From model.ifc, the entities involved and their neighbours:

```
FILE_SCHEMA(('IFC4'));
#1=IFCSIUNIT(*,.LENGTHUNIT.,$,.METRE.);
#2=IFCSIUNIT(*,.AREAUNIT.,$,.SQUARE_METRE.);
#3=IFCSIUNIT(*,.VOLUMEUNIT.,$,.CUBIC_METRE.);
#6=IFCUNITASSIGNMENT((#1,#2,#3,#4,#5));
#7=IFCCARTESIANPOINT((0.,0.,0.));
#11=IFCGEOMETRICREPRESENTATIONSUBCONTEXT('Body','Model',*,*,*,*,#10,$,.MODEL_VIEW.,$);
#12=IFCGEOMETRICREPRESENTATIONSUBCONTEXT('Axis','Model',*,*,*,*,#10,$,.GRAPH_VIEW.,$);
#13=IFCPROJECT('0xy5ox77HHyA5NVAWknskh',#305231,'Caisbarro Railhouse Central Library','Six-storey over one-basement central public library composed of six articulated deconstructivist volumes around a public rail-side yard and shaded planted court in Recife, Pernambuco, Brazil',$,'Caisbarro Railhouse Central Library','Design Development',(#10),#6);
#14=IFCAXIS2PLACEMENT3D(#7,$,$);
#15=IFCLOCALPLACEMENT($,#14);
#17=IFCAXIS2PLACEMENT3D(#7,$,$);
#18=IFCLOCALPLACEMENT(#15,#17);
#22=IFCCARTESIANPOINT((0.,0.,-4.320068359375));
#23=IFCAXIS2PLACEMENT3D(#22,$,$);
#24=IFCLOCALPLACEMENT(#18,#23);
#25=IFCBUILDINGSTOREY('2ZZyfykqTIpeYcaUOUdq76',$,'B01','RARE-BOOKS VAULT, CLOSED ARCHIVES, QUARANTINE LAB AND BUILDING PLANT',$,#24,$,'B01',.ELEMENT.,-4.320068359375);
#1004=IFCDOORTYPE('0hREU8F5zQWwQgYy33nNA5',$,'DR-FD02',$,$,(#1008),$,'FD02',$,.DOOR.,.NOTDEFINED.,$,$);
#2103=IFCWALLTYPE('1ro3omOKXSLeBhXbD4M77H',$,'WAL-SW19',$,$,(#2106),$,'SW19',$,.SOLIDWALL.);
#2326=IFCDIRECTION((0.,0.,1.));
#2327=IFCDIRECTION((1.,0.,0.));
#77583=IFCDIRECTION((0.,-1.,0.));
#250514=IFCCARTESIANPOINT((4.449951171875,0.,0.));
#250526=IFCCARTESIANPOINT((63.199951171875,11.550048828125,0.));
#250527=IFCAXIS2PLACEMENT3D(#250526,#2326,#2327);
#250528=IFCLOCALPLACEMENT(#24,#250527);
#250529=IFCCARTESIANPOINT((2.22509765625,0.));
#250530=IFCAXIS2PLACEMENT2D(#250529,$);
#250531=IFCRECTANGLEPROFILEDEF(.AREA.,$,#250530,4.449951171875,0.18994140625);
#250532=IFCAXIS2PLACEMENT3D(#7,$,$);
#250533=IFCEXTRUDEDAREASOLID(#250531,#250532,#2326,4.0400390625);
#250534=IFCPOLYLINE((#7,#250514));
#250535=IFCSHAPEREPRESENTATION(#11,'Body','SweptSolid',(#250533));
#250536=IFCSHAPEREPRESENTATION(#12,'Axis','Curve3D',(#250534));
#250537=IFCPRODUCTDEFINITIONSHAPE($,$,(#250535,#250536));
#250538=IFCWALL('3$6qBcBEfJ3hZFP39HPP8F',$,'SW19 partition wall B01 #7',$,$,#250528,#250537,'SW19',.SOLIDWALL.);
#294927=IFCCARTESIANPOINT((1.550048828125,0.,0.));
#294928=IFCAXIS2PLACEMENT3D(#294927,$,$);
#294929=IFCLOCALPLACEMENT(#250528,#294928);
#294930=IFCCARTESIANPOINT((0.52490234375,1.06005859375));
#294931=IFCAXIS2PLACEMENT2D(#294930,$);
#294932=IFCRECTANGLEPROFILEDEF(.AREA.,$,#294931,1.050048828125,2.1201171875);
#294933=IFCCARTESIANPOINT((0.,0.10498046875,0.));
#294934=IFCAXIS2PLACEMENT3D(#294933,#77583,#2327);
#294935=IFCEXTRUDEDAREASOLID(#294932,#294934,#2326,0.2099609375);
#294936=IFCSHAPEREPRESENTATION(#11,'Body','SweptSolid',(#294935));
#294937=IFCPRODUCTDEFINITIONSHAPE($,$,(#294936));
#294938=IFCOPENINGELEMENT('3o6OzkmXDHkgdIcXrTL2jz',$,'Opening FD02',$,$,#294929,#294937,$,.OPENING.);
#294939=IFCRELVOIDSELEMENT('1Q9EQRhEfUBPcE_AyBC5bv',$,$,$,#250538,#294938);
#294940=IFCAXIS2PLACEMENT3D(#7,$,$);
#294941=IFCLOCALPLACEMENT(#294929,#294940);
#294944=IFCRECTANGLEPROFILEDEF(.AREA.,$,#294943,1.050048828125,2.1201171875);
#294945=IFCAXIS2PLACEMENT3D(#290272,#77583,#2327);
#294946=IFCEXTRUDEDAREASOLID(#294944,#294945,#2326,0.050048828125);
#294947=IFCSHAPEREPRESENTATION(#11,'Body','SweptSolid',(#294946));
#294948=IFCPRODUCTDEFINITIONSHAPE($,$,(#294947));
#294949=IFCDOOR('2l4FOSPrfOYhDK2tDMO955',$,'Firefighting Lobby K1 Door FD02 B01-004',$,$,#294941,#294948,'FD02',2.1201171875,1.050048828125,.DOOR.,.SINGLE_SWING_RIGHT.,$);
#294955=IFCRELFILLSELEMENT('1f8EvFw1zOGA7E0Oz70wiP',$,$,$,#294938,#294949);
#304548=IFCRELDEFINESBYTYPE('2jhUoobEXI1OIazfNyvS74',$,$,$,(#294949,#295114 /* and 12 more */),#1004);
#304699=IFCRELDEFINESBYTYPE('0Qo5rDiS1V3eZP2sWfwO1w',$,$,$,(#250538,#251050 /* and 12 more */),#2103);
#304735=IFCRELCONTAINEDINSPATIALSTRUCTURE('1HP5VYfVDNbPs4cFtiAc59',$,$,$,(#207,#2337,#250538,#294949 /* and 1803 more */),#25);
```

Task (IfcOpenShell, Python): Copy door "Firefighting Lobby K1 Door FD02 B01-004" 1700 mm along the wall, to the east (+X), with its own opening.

```python
import ifcopenshell
import ifcopenshell.api.feature
import ifcopenshell.api.geometry
import ifcopenshell.api.root
import ifcopenshell.geom
import ifcopenshell.util.element
import ifcopenshell.util.placement
import ifcopenshell.util.shape
import ifcopenshell.util.unit

model = ifcopenshell.open("model.ifc")
unit_scale = ifcopenshell.util.unit.calculate_unit_scale(model)
settings = ifcopenshell.geom.settings()


def volume(element):
    """Net volume in cubic metres, openings subtracted."""
    shape = ifcopenshell.geom.create_shape(settings, element)
    return ifcopenshell.util.shape.get_volume(shape.geometry)


door = model.by_guid("2l4FOSPrfOYhDK2tDMO955")
opening = door.FillsVoids[0].RelatingOpeningElement
wall = opening.VoidsElements[0].RelatingBuildingElement
before = volume(wall)
shift = ifcopenshell.util.placement.get_local_placement(wall.ObjectPlacement)[:3, 0] * 1.7 / unit_scale

# copy_class copies the void relationship, type, container and properties, but no geometry.
new_opening = ifcopenshell.api.root.copy_class(model, product=opening)
new_opening.Representation = ifcopenshell.util.element.copy_deep(
    model, opening.Representation, exclude=["IfcGeometricRepresentationContext", "IfcRepresentationMap"]
)
new_door = ifcopenshell.api.root.copy_class(model, product=door)
new_door.Representation = ifcopenshell.util.element.copy_deep(
    model, door.Representation, exclude=["IfcGeometricRepresentationContext", "IfcRepresentationMap"]
)
new_door.Tag = None
ifcopenshell.api.feature.add_filling(model, opening=new_opening, element=new_door)

for old, new in ((opening, new_opening), (door, new_door)):
    matrix = ifcopenshell.util.placement.get_local_placement(old.ObjectPlacement)
    matrix[:3, 3] += shift
    ifcopenshell.api.geometry.edit_object_placement(model, product=new, matrix=matrix, is_si=False)

after = volume(wall)

print(f"wall volume {before:.3f} -> {after:.3f} m3")

model.write("model_edited.ifc")
```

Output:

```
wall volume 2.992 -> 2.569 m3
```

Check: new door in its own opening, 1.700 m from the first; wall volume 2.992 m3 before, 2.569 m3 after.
